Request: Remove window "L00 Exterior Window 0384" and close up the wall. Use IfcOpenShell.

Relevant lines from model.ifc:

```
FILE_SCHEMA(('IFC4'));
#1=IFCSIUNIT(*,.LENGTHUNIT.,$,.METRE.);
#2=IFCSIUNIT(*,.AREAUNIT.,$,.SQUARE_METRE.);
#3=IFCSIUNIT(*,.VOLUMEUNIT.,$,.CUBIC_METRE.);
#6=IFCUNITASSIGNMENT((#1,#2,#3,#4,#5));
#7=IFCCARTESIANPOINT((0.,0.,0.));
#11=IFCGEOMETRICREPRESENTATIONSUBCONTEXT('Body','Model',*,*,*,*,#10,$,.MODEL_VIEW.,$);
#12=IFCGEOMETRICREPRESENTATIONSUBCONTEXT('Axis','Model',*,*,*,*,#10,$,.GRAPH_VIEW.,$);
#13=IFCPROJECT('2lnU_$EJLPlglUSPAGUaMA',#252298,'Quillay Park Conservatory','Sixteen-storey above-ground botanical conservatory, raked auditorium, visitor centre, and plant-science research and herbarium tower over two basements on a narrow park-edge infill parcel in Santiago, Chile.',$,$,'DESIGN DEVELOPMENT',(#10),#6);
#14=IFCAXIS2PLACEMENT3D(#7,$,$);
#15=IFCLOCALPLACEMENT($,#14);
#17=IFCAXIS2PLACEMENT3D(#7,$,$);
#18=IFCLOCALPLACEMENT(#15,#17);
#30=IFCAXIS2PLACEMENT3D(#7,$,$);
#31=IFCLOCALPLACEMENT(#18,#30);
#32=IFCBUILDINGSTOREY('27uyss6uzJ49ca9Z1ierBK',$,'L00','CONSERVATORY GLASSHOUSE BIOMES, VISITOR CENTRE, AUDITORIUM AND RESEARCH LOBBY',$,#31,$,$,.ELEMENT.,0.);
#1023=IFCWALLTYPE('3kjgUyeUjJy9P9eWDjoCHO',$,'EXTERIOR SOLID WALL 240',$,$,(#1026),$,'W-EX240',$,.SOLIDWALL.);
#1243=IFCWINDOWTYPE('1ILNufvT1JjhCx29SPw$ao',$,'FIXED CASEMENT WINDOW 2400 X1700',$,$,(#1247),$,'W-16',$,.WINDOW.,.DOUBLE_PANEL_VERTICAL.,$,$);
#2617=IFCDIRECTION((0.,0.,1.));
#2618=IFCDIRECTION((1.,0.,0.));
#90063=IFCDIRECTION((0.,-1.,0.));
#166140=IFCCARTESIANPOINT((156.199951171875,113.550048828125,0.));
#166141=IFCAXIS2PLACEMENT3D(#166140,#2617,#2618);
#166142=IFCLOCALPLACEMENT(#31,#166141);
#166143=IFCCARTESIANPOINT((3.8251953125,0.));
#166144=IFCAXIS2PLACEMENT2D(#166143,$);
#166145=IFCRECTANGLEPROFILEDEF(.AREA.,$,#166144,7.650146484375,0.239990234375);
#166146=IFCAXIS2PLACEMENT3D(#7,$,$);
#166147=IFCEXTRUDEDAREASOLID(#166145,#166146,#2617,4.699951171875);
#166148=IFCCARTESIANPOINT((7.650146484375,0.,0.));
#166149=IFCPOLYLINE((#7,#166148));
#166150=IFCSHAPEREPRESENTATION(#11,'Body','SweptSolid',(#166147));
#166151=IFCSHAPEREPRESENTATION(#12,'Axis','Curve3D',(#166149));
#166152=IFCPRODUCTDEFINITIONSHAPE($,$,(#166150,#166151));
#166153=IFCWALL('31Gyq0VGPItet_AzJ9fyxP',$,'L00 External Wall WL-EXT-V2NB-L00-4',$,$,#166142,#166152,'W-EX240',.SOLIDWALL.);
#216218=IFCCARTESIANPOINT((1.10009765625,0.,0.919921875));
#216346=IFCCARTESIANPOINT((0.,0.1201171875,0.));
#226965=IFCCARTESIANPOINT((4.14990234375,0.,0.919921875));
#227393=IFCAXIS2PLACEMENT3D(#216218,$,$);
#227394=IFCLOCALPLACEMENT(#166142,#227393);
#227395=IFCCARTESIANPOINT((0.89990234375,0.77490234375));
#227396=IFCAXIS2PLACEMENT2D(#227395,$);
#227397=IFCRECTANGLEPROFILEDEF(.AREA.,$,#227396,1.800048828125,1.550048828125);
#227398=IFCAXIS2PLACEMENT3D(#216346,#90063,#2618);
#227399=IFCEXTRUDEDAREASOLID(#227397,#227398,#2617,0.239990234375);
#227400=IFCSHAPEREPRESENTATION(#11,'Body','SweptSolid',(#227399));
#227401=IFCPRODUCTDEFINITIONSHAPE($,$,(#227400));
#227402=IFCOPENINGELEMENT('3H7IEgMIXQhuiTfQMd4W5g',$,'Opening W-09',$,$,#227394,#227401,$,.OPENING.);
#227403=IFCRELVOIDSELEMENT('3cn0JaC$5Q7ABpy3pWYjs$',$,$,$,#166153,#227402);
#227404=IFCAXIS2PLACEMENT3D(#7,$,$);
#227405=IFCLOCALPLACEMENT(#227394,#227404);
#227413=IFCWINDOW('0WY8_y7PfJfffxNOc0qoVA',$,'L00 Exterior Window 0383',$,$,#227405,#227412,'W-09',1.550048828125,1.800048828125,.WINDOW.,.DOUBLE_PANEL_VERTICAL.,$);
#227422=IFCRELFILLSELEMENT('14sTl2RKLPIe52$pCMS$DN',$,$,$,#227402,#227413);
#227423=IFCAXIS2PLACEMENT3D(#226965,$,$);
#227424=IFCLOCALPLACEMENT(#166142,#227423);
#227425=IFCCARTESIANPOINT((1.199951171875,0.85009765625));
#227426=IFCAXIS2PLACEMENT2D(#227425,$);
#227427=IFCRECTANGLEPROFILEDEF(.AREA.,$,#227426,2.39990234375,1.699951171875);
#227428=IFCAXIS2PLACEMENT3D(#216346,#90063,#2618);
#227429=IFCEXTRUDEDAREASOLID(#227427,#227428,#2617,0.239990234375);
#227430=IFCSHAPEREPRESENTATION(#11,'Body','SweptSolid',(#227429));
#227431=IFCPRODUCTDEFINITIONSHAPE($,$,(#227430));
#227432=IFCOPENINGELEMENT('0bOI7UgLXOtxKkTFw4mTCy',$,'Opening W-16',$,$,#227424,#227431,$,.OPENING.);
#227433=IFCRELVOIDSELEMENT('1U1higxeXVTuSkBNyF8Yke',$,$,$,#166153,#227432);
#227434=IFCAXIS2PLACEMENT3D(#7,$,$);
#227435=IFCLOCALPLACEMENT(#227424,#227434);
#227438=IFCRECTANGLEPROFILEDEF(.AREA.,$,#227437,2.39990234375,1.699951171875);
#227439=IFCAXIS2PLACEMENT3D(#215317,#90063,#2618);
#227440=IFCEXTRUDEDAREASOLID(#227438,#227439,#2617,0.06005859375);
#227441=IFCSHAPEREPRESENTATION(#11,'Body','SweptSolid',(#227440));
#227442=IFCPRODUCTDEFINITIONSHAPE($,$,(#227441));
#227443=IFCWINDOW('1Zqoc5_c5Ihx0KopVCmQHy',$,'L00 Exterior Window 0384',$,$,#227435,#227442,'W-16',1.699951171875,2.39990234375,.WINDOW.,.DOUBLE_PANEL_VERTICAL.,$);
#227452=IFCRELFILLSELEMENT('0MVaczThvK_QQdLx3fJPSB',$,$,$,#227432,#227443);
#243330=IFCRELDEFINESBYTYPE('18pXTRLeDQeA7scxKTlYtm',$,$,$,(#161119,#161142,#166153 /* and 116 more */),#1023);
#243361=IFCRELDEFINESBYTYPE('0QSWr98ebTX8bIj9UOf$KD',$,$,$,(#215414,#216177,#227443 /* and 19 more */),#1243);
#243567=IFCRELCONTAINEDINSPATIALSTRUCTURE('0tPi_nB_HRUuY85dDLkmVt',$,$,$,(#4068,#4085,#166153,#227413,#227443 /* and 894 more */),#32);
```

```python
import ifcopenshell
import ifcopenshell.api.feature
import ifcopenshell.api.root
import ifcopenshell.geom
import ifcopenshell.util.shape

model = ifcopenshell.open("model.ifc")
settings = ifcopenshell.geom.settings()


def volume(element):
    """Net volume in cubic metres, openings subtracted."""
    shape = ifcopenshell.geom.create_shape(settings, element)
    return ifcopenshell.util.shape.get_volume(shape.geometry)


window = model.by_guid("1Zqoc5_c5Ihx0KopVCmQHy")
opening = window.FillsVoids[0].RelatingOpeningElement
wall = opening.VoidsElements[0].RelatingBuildingElement
before = volume(wall)

ifcopenshell.api.root.remove_product(model, product=window)
ifcopenshell.api.feature.remove_feature(model, feature=opening)

after = volume(wall)

print(f"wall volume {before:.3f} -> {after:.3f} m3")

model.write("model_edited.ifc")
```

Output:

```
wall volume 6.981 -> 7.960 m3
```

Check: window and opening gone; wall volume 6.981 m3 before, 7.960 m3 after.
